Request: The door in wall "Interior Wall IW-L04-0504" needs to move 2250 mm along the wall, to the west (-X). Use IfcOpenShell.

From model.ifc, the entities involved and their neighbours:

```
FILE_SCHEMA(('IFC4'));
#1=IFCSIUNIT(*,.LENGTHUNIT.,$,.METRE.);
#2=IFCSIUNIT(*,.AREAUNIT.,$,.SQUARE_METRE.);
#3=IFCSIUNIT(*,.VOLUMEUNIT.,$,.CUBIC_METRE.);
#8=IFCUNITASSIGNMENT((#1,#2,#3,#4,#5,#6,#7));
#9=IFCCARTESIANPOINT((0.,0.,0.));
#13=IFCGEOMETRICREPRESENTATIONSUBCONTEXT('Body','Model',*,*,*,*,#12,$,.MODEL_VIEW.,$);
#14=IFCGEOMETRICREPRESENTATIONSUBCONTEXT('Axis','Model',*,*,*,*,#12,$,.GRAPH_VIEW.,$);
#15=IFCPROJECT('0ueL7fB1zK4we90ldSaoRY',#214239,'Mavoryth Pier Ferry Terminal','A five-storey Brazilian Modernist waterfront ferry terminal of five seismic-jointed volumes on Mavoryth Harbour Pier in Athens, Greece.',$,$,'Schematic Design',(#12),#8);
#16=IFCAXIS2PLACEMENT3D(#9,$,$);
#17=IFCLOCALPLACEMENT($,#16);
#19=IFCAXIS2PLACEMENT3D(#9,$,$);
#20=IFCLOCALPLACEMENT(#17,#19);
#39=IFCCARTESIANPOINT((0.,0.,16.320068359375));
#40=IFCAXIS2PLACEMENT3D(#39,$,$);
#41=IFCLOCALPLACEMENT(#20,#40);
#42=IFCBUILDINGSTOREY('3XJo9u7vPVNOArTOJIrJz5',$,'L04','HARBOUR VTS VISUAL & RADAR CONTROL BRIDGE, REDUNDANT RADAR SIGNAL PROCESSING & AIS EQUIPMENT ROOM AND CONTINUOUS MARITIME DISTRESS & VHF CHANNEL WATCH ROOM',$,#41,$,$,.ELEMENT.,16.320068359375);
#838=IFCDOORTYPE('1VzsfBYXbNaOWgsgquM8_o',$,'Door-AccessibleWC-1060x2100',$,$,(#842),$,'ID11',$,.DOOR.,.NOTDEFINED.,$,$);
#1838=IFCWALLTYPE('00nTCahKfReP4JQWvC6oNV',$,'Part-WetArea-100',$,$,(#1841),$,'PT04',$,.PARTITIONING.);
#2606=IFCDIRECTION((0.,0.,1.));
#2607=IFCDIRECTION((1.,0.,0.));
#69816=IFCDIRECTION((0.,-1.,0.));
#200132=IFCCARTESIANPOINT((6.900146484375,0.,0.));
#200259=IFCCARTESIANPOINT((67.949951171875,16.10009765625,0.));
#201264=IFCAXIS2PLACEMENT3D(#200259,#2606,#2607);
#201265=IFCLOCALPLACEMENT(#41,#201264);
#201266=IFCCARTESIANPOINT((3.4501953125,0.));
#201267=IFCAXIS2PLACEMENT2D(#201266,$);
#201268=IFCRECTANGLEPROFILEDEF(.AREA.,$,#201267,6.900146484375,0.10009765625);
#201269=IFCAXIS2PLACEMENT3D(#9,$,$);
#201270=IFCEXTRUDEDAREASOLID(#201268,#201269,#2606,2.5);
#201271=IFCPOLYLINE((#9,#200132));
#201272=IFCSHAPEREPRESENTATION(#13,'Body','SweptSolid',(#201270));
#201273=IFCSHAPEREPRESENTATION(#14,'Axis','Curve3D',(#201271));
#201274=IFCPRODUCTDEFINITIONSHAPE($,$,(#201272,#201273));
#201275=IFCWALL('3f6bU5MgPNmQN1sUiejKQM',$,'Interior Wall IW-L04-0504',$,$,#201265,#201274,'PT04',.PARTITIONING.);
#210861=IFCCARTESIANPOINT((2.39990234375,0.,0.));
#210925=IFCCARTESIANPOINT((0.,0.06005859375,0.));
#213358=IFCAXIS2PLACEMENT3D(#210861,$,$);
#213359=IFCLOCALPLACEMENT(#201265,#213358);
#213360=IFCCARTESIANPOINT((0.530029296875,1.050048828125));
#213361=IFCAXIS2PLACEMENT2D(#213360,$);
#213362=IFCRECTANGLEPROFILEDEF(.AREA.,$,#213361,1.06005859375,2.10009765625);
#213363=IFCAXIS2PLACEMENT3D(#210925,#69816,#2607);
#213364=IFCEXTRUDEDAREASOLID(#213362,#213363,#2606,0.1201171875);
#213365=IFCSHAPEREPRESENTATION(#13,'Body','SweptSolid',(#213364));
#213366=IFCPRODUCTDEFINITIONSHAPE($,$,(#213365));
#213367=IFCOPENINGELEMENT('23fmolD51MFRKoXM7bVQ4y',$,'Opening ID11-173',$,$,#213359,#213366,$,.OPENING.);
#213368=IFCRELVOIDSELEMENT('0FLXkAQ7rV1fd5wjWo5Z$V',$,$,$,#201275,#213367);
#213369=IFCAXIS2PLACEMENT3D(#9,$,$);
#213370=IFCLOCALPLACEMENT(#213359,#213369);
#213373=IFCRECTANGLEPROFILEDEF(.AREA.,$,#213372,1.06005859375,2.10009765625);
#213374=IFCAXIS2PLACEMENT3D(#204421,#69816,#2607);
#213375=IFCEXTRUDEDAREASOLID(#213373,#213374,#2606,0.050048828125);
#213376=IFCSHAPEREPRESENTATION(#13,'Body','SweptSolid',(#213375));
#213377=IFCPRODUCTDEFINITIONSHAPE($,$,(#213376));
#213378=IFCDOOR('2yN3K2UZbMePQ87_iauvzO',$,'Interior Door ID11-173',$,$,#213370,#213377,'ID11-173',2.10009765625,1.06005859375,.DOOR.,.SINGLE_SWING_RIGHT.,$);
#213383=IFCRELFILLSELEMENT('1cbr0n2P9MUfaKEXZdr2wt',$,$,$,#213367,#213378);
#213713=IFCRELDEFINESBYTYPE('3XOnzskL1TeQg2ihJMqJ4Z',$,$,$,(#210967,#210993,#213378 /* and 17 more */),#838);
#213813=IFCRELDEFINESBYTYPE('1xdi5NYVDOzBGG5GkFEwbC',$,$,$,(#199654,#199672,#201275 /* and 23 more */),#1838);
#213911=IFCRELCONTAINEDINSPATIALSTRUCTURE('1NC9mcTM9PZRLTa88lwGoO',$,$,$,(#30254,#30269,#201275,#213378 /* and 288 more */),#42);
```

```python
import ifcopenshell
import ifcopenshell.api.geometry
import ifcopenshell.util.placement

model = ifcopenshell.open("model.ifc")

door = model.by_guid("2yN3K2UZbMePQ87_iauvzO")
opening = door.FillsVoids[0].RelatingOpeningElement
wall = opening.VoidsElements[0].RelatingBuildingElement

wall_matrix = ifcopenshell.util.placement.get_local_placement(wall.ObjectPlacement)
shift = wall_matrix[:3, 0] * -2.25
before = ifcopenshell.util.placement.get_local_placement(door.ObjectPlacement)[:3, 3].copy()

# The door is placed relative to its opening, so it follows when the opening moves.
matrix = ifcopenshell.util.placement.get_local_placement(opening.ObjectPlacement)
matrix[:3, 3] += shift
ifcopenshell.api.geometry.edit_object_placement(
    model, product=opening, matrix=matrix, is_si=False, should_transform_children=True
)

after = ifcopenshell.util.placement.get_local_placement(door.ObjectPlacement)[:3, 3]
print("door moved by", (after - before).round(3) + 0.0)

model.write("model_rev.ifc")
```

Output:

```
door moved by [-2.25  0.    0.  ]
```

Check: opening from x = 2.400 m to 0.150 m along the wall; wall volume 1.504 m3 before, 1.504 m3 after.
